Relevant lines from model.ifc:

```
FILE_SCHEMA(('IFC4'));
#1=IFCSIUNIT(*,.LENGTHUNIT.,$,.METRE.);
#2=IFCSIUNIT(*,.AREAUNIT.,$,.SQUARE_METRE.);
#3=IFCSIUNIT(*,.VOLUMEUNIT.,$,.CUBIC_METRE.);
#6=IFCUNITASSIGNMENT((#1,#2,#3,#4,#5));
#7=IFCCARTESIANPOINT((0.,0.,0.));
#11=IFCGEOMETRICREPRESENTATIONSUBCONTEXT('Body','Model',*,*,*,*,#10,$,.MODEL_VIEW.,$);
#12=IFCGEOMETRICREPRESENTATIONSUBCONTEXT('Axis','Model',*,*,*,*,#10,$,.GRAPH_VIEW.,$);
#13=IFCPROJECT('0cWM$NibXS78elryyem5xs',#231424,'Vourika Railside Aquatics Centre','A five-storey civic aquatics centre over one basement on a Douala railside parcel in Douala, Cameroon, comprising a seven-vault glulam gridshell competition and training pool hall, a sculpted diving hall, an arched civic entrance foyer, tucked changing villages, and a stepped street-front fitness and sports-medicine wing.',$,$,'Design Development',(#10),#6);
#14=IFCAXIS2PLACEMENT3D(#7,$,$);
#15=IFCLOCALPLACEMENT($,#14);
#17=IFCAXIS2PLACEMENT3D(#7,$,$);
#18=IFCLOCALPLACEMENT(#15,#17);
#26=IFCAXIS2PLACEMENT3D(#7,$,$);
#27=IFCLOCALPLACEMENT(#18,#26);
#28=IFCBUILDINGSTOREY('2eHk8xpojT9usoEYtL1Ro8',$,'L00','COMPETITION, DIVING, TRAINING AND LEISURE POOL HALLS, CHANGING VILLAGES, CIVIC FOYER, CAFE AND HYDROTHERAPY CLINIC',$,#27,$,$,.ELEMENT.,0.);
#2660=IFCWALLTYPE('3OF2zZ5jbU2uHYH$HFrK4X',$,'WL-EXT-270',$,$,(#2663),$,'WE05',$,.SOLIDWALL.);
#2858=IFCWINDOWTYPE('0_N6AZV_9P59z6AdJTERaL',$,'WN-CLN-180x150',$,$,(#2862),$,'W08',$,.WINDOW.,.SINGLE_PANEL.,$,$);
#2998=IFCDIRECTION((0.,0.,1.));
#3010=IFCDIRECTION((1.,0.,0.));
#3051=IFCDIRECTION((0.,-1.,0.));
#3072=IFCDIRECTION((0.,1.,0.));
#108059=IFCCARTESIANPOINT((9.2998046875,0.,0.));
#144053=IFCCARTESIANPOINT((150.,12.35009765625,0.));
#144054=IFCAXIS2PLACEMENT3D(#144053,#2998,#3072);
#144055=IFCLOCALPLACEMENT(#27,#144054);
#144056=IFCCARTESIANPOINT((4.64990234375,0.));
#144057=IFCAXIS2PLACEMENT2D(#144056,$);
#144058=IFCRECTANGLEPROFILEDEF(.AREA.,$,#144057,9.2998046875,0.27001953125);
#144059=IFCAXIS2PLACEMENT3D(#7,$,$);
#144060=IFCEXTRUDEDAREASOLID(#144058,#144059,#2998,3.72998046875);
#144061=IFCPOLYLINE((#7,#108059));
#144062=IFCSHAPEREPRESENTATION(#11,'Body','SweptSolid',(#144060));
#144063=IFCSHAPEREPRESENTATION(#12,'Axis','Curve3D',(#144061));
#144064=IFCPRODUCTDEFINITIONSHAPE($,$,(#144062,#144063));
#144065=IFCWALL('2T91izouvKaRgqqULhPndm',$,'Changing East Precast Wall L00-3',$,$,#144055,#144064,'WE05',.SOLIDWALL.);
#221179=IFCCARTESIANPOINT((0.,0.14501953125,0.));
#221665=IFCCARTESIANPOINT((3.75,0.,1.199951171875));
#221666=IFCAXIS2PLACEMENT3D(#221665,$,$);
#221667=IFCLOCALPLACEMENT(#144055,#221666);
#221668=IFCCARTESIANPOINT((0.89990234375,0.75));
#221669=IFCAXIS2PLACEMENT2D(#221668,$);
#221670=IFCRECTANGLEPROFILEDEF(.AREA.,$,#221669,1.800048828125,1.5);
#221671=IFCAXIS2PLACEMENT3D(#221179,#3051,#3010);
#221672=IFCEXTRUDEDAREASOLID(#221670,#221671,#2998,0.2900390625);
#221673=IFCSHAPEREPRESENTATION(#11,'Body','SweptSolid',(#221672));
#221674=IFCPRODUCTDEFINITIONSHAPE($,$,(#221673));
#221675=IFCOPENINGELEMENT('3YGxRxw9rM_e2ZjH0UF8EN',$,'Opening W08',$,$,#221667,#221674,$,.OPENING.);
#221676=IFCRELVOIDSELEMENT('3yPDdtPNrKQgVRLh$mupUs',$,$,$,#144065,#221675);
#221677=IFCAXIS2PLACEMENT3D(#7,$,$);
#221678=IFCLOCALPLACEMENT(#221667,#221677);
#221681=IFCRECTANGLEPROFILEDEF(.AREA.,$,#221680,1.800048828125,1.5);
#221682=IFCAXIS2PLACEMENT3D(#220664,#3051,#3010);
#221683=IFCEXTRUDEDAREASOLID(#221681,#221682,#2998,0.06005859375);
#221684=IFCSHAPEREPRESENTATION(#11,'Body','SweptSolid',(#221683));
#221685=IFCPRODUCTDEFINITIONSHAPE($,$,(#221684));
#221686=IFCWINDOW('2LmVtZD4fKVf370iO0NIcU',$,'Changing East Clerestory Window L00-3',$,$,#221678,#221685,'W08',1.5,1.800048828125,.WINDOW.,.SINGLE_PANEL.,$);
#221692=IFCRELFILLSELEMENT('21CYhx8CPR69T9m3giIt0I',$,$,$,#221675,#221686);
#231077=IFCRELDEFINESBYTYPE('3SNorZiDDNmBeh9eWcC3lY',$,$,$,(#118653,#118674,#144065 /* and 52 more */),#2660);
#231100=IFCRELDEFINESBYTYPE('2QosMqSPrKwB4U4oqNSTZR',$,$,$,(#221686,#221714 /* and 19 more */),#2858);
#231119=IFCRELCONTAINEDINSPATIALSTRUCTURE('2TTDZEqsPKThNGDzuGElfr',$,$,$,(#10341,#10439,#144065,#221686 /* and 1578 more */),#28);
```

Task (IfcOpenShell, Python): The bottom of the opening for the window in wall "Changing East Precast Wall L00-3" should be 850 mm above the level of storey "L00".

```python
import numpy as np
import ifcopenshell
import ifcopenshell.api.geometry
import ifcopenshell.geom
import ifcopenshell.util.element
import ifcopenshell.util.placement
import ifcopenshell.util.shape
import ifcopenshell.util.unit

model = ifcopenshell.open("model.ifc")
unit_scale = ifcopenshell.util.unit.calculate_unit_scale(model)

window = model.by_guid("2LmVtZD4fKVf370iO0NIcU")
opening = window.FillsVoids[0].RelatingOpeningElement
storey = ifcopenshell.util.element.get_container(window, ifc_class="IfcBuildingStorey")
level = ifcopenshell.util.placement.get_local_placement(storey.ObjectPlacement)[2, 3]

# The opening's origin need not be at the sill, so measure its lowest point.
shape = ifcopenshell.geom.create_shape(ifcopenshell.geom.settings(), opening)
bottom = ifcopenshell.util.shape.get_shape_bottom_elevation(shape, shape.geometry) / unit_scale
dz = level + 0.85 - bottom

shift = np.array([0.0, 0.0, dz])
# The window is placed relative to its opening, so it follows when the opening moves.
matrix = ifcopenshell.util.placement.get_local_placement(opening.ObjectPlacement)
matrix[:3, 3] += shift
ifcopenshell.api.geometry.edit_object_placement(
    model, product=opening, matrix=matrix, is_si=False, should_transform_children=True
)

print(f"moved by {dz * unit_scale:+.3f} m")

model.write("model_v2.ifc")
```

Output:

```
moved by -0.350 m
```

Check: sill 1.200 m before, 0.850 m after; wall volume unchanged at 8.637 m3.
